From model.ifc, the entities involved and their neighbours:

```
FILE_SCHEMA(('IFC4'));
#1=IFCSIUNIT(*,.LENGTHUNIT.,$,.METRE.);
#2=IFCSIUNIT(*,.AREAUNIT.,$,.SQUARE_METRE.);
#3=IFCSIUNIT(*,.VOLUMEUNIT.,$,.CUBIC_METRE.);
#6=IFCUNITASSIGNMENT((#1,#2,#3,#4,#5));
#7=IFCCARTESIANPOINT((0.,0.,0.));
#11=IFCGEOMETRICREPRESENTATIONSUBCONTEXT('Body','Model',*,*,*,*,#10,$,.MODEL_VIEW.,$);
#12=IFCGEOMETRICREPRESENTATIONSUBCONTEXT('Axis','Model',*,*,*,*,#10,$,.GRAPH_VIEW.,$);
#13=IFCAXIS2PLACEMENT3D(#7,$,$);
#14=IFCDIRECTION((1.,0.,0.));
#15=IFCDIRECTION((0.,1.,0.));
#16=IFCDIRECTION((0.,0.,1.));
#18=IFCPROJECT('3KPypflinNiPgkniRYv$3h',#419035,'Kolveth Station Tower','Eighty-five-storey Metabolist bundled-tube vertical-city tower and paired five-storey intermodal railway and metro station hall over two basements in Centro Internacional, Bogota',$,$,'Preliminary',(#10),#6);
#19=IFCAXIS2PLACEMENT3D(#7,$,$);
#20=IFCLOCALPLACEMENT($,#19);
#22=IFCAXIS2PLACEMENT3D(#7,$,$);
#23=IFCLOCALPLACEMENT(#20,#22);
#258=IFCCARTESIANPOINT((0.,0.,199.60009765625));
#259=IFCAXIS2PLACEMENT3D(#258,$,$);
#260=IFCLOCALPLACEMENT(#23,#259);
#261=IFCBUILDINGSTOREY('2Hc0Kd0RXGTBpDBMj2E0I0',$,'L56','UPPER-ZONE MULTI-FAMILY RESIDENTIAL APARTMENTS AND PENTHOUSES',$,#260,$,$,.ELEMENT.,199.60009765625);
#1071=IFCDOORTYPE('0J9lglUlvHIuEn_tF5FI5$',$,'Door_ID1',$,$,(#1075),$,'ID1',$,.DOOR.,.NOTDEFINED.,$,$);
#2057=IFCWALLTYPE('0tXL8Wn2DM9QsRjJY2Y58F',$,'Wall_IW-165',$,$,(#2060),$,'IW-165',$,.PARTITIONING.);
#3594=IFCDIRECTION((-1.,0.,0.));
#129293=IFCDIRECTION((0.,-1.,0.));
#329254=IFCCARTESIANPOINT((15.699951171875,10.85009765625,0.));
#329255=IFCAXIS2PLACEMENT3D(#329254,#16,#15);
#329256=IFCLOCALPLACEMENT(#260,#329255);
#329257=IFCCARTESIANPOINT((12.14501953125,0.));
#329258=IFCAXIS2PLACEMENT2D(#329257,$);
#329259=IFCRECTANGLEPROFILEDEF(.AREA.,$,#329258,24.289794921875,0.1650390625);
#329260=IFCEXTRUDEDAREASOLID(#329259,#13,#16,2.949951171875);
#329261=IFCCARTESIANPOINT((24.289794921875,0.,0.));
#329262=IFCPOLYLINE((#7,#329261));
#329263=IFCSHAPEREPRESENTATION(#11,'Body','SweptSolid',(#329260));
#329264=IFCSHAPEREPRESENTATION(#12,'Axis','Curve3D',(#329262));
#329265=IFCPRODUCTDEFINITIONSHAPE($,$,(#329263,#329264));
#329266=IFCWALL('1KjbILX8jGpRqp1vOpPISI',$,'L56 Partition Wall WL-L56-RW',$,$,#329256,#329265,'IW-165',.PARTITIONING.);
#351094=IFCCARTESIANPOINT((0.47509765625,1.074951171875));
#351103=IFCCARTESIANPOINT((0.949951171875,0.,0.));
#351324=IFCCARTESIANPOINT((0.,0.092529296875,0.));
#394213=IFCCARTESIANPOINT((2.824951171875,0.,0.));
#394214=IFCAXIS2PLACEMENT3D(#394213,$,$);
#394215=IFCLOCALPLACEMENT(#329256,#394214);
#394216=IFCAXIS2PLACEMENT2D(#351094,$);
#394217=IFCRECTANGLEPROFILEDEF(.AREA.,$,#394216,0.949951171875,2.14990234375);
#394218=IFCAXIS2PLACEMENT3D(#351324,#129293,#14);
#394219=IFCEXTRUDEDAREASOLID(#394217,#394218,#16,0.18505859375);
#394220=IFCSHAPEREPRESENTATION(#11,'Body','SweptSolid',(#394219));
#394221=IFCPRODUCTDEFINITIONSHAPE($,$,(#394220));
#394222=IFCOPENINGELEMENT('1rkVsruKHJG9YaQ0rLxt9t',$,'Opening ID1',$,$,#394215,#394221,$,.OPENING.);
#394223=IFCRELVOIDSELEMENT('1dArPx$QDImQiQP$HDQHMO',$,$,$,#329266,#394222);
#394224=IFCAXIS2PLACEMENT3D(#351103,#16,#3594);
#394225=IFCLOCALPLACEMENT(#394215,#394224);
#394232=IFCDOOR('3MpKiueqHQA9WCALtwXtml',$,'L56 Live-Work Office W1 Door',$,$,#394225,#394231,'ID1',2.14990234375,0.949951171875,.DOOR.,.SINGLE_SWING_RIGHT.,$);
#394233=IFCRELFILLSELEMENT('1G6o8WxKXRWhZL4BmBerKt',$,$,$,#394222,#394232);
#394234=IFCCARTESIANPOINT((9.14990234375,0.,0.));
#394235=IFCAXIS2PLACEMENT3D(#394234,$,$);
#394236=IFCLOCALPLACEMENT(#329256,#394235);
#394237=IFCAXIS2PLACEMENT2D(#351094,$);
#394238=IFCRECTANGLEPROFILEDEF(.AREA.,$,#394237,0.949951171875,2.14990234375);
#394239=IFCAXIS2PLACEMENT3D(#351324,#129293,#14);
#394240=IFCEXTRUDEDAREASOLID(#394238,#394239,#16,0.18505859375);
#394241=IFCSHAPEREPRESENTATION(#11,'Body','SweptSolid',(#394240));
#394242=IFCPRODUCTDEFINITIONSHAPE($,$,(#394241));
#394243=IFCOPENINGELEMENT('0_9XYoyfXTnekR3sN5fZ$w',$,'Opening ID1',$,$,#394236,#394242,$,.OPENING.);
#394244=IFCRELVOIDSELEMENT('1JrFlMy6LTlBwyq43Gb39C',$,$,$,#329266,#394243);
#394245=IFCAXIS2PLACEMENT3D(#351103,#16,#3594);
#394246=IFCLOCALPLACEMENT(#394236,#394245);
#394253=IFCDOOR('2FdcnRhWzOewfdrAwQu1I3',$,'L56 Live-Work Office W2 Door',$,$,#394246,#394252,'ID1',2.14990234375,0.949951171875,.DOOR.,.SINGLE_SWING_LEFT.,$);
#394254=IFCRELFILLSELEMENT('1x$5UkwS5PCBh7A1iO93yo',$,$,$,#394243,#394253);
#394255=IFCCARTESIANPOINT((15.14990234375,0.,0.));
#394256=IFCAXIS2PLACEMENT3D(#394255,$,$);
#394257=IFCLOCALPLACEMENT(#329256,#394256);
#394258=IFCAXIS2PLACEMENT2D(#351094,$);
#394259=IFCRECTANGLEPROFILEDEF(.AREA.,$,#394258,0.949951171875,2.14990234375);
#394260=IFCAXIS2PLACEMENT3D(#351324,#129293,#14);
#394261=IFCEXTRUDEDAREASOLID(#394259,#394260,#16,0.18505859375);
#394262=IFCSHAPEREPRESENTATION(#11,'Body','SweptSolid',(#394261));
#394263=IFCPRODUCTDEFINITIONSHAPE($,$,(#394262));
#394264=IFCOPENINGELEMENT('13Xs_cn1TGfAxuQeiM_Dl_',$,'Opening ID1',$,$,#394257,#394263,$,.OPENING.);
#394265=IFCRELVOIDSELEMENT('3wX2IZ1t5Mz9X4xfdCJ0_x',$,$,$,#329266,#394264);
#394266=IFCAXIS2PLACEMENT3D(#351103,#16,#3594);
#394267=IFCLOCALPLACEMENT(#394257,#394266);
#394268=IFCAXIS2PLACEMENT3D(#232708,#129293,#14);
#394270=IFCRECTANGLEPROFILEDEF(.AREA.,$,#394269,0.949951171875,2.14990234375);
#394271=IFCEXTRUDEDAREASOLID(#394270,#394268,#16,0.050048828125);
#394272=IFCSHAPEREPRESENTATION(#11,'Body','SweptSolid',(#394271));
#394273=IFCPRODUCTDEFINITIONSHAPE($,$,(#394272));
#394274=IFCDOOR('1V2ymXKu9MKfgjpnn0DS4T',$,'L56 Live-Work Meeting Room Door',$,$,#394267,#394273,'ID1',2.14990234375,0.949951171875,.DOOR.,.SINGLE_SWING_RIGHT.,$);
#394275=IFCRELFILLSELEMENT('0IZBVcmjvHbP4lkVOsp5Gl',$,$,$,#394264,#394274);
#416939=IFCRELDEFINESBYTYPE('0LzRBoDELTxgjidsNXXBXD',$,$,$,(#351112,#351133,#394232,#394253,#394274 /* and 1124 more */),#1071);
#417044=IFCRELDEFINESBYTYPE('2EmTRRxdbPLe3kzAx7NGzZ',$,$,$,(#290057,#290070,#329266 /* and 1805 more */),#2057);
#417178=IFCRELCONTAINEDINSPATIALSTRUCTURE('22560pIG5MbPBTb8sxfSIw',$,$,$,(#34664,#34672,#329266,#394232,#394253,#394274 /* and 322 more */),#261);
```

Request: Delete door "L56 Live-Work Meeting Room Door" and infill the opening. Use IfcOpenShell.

```python
import ifcopenshell
import ifcopenshell.api.feature
import ifcopenshell.api.root
import ifcopenshell.geom
import ifcopenshell.util.shape

model = ifcopenshell.open("model.ifc")
settings = ifcopenshell.geom.settings()


def volume(element):
    """Net volume in cubic metres, openings subtracted."""
    shape = ifcopenshell.geom.create_shape(settings, element)
    return ifcopenshell.util.shape.get_volume(shape.geometry)


door = model.by_guid("1V2ymXKu9MKfgjpnn0DS4T")
opening = door.FillsVoids[0].RelatingOpeningElement
wall = opening.VoidsElements[0].RelatingBuildingElement
before = volume(wall)

ifcopenshell.api.root.remove_product(model, product=door)
ifcopenshell.api.feature.remove_feature(model, feature=opening)

after = volume(wall)

print(f"wall volume {before:.3f} -> {after:.3f} m3")

model.write("model_v2.ifc")
```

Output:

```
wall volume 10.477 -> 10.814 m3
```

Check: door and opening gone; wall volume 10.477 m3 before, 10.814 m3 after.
